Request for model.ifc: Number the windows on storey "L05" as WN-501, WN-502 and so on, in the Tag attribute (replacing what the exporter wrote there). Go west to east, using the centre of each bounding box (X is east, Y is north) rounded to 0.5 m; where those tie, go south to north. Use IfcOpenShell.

First a look at what the model holds.

```python
import ifcopenshell
import ifcopenshell.util.element
import ifcopenshell.util.placement

model = ifcopenshell.open("model.ifc")
print(model.schema)
storey = next(s for s in model.by_type("IfcBuildingStorey") if s.Name == "L05")
windows = [e for e in ifcopenshell.util.element.get_decomposition(storey) if e.is_a("IfcWindow")]
for e in sorted(windows, key=lambda e: e.id()):
    origin = ifcopenshell.util.placement.get_local_placement(e.ObjectPlacement)[:3, 3]
    print(e.id(), e.Tag, e.Name, origin.round(2) + 0.0, sep=" | ")
```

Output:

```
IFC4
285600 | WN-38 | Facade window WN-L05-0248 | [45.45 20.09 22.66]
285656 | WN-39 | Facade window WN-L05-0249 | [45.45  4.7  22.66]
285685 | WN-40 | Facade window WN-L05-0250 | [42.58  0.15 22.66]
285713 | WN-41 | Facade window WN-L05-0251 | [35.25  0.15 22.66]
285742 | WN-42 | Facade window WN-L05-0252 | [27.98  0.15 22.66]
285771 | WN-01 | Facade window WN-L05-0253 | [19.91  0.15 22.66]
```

```python
import ifcopenshell
import ifcopenshell.geom
import ifcopenshell.util.element
import ifcopenshell.util.shape

model = ifcopenshell.open("model.ifc")
settings = ifcopenshell.geom.settings()
settings.set("use-world-coords", True)


def centre(element):
    shape = ifcopenshell.geom.create_shape(settings, element)
    return ifcopenshell.util.shape.get_bbox_centroid(shape.geometry)


storey = next(s for s in model.by_type("IfcBuildingStorey") if s.Name == "L05")
windows = [e for e in ifcopenshell.util.element.get_decomposition(storey) if e.is_a("IfcWindow")]

# Insertion points can sit at a corner or the storey origin, so sort by the geometry (in metres).
centres = {e: centre(e) for e in windows}
windows.sort(key=lambda e: (round(centres[e][0] / 0.5), centres[e][1]))

for i, e in enumerate(windows, start=1):
    number = f"WN-5{i:02d}"
    e.Tag = number
    print(e.id(), number)

model.write("model_rev.ifc")
```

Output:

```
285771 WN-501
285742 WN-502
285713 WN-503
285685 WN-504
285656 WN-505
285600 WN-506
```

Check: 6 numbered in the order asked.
